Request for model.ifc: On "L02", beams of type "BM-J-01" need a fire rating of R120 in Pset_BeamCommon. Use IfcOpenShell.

First a look at what the model holds.

```python
import ifcopenshell
import ifcopenshell.util.element

model = ifcopenshell.open("model.ifc")
print(model.schema)
storey = next(s for s in model.by_type("IfcBuildingStorey") if s.Name == "L02")
beams = [e for e in ifcopenshell.util.element.get_decomposition(storey) if e.is_a("IfcBeam")]
seen = {}
for e in beams:
    element_type = ifcopenshell.util.element.get_type(e)
    key = (element_type.Name if element_type != e and element_type else None, ifcopenshell.util.element.get_pset(e, "Pset_BeamCommon", "FireRating"))
    seen[key] = seen.get(key, 0) + 1
for (name, value), count in sorted(seen.items(), key=str):
    print(count, "x", name, "|", value)
```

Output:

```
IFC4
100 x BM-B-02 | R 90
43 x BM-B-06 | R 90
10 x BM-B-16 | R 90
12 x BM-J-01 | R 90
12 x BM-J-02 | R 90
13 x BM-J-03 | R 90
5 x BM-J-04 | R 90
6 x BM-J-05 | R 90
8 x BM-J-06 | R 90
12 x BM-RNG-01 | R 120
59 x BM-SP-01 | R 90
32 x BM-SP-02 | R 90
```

```python
import ifcopenshell
import ifcopenshell.api.pset
import ifcopenshell.util.element

model = ifcopenshell.open("model.ifc")

storey = next(s for s in model.by_type("IfcBuildingStorey") if s.Name == "L02")
beams = [e for e in ifcopenshell.util.element.get_decomposition(storey) if e.is_a("IfcBeam")]

count = 0
for e in beams:
    element_type = ifcopenshell.util.element.get_type(e)
    if element_type in (None, e) or element_type.Name != "BM-J-01":
        continue
    # add_pset returns the element's existing set when there is one.
    pset = ifcopenshell.api.pset.add_pset(model, product=e, name="Pset_BeamCommon")
    ifcopenshell.api.pset.edit_pset(model, pset=pset, properties={"FireRating": "R120"})
    count += 1

print(count, "beams updated")

model.write("model-out.ifc")
```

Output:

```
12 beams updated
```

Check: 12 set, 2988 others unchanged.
